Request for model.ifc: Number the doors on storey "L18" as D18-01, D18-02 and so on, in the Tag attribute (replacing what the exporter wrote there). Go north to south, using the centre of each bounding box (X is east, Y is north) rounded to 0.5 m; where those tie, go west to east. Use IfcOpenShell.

First a look at what the model holds.

```python
import ifcopenshell
import ifcopenshell.util.element
import ifcopenshell.util.placement

model = ifcopenshell.open("model.ifc")
print(model.schema)
storey = next(s for s in model.by_type("IfcBuildingStorey") if s.Name == "L18")
doors = [e for e in ifcopenshell.util.element.get_decomposition(storey) if e.is_a("IfcDoor")]
for e in sorted(doors, key=lambda e: e.id()):
    origin = ifcopenshell.util.placement.get_local_placement(e.ObjectPlacement)[:3, 3]
    print(e.id(), e.Tag, e.Name, origin.round(2) + 0.0, sep=" | ")
```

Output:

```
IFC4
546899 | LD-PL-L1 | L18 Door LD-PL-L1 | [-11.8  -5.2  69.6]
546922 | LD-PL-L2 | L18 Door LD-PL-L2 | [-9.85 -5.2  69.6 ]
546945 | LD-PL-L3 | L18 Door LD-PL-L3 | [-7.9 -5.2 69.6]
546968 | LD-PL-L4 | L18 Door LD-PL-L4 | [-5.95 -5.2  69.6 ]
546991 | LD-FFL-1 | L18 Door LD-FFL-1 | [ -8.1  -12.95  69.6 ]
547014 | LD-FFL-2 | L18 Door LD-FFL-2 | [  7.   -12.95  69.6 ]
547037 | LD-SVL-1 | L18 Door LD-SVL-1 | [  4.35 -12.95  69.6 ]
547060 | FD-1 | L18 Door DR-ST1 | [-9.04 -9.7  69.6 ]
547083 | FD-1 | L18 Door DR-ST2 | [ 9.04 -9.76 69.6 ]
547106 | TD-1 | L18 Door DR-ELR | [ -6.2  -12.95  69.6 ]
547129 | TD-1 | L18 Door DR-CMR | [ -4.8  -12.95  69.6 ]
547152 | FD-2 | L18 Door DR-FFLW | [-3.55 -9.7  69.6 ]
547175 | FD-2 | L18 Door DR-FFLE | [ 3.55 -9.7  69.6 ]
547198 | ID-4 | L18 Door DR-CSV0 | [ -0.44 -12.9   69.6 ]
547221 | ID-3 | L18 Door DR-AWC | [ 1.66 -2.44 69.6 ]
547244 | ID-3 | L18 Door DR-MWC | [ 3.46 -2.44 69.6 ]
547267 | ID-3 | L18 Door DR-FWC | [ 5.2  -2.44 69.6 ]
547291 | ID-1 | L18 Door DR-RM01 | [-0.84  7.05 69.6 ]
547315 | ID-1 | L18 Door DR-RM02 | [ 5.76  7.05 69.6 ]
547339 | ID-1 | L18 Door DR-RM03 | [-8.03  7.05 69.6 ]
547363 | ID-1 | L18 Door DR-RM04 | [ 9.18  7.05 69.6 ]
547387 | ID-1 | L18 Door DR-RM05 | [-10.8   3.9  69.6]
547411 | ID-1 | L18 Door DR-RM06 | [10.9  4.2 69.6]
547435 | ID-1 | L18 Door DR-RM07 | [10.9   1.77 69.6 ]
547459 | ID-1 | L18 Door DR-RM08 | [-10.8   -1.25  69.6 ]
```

```python
import ifcopenshell
import ifcopenshell.geom
import ifcopenshell.util.element
import ifcopenshell.util.shape

model = ifcopenshell.open("model.ifc")
settings = ifcopenshell.geom.settings()
settings.set("use-world-coords", True)


def centre(element):
    shape = ifcopenshell.geom.create_shape(settings, element)
    return ifcopenshell.util.shape.get_bbox_centroid(shape.geometry)


storey = next(s for s in model.by_type("IfcBuildingStorey") if s.Name == "L18")
doors = [e for e in ifcopenshell.util.element.get_decomposition(storey) if e.is_a("IfcDoor")]

# Insertion points can sit at a corner or the storey origin, so sort by the geometry (in metres).
centres = {e: centre(e) for e in doors}
doors.sort(key=lambda e: (-round(centres[e][1] / 0.5), centres[e][0]))

for i, e in enumerate(doors, start=1):
    number = f"D18-{i:02d}"
    e.Tag = number
    print(e.id(), number)

model.write("model_edited.ifc")
```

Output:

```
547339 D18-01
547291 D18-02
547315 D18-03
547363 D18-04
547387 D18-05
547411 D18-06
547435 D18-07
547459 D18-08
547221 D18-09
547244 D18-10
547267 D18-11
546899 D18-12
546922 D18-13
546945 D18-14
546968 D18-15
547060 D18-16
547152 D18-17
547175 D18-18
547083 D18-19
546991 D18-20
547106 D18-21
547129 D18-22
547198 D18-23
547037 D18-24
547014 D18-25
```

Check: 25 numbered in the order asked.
